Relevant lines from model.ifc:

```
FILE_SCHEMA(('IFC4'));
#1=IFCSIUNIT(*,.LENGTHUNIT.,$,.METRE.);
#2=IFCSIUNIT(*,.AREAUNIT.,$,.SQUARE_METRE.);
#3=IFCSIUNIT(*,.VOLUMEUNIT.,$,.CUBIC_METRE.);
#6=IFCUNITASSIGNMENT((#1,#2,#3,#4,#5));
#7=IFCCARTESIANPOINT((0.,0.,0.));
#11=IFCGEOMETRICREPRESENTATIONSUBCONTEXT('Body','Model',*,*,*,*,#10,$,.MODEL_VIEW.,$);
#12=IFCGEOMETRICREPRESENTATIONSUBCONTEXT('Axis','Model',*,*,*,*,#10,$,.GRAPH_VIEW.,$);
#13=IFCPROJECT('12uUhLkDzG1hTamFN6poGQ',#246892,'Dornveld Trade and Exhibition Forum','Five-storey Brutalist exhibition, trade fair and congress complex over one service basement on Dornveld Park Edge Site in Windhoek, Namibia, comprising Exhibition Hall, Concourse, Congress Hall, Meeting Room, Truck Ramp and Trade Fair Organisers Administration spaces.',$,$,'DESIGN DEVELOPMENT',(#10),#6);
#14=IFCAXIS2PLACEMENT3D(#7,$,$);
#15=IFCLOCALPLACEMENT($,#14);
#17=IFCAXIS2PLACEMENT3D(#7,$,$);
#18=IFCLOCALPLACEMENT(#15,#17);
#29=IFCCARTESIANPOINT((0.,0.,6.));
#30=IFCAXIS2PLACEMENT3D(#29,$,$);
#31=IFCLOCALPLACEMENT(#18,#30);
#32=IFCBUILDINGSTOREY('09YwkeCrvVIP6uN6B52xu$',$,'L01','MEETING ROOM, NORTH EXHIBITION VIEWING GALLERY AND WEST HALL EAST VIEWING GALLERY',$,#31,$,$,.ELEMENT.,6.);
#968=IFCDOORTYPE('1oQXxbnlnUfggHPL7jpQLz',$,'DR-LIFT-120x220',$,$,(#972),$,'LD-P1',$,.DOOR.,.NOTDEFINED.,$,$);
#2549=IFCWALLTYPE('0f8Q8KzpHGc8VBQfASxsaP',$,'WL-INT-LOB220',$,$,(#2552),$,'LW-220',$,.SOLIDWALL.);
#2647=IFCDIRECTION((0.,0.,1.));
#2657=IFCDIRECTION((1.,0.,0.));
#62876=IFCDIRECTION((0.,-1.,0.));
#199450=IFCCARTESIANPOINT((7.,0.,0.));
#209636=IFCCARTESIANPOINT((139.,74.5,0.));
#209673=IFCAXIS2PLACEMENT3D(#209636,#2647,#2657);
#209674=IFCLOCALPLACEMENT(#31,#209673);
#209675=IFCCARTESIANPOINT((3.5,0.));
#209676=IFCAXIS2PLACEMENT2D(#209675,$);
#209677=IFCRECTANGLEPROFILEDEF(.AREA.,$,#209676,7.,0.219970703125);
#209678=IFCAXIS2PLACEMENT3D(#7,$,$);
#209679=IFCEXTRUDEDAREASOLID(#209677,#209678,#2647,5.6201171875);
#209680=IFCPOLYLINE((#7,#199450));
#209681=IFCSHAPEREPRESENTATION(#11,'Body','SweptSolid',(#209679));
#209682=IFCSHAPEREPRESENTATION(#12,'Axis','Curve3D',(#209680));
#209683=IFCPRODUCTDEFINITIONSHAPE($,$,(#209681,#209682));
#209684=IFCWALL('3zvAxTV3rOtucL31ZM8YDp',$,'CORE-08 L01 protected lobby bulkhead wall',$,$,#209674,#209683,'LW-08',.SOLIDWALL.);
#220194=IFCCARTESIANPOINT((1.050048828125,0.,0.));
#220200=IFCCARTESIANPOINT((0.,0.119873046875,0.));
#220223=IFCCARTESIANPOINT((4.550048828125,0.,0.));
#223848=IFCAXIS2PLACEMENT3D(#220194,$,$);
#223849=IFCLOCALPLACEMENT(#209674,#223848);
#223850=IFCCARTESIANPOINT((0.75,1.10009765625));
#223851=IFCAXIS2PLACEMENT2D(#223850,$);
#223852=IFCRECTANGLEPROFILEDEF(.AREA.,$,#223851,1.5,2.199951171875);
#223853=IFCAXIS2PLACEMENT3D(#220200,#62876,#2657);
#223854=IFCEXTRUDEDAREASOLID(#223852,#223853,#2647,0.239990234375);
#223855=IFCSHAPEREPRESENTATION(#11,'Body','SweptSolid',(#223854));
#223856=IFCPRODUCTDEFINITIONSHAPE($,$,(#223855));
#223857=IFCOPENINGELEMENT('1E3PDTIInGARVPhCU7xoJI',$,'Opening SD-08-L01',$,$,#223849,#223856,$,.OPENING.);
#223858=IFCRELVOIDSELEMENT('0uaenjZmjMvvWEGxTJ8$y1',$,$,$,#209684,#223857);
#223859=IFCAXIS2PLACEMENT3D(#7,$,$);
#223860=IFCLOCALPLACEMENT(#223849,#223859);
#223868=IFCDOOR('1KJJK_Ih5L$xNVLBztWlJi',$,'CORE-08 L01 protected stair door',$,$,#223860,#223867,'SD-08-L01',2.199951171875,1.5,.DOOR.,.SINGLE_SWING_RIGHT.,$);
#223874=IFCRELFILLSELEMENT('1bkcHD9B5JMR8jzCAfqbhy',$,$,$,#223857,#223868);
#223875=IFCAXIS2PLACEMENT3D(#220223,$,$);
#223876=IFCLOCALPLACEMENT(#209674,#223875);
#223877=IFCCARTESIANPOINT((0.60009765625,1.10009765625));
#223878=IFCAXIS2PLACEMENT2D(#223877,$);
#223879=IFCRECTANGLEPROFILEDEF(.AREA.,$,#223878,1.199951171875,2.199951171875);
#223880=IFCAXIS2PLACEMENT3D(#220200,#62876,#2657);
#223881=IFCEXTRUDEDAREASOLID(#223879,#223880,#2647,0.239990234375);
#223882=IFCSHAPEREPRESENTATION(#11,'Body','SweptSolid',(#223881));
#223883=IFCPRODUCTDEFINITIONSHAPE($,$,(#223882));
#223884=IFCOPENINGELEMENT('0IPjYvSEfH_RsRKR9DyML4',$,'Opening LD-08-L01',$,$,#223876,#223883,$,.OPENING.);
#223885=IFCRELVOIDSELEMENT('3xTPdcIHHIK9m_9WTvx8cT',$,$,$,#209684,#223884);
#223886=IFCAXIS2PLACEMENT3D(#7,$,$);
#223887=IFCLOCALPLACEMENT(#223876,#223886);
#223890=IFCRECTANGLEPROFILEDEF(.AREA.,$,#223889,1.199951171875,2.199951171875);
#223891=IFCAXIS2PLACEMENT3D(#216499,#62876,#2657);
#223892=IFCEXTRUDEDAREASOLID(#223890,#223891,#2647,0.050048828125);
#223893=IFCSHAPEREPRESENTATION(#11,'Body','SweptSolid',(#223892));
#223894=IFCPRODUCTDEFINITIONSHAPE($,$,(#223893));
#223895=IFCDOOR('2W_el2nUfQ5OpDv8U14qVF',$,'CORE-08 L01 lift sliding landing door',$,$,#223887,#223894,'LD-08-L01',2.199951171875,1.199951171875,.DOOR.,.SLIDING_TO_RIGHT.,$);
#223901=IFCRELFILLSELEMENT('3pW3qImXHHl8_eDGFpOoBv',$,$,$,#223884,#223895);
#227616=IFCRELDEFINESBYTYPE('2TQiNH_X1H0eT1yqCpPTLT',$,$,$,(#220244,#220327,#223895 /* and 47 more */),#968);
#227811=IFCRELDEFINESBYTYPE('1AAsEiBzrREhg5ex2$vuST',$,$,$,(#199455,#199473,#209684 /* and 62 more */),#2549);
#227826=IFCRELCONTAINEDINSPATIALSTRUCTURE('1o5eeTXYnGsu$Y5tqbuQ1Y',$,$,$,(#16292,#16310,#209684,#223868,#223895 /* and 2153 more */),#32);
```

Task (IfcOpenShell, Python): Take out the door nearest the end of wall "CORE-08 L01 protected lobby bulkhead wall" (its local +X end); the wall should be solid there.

```python
import ifcopenshell
import ifcopenshell.api.feature
import ifcopenshell.api.root
import ifcopenshell.geom
import ifcopenshell.util.shape

model = ifcopenshell.open("model.ifc")
settings = ifcopenshell.geom.settings()


def volume(element):
    """Net volume in cubic metres, openings subtracted."""
    shape = ifcopenshell.geom.create_shape(settings, element)
    return ifcopenshell.util.shape.get_volume(shape.geometry)


door = model.by_guid("2W_el2nUfQ5OpDv8U14qVF")
opening = door.FillsVoids[0].RelatingOpeningElement
wall = opening.VoidsElements[0].RelatingBuildingElement
before = volume(wall)

ifcopenshell.api.root.remove_product(model, product=door)
ifcopenshell.api.feature.remove_feature(model, feature=opening)

after = volume(wall)

print(f"wall volume {before:.3f} -> {after:.3f} m3")

model.write("model_v2.ifc")
```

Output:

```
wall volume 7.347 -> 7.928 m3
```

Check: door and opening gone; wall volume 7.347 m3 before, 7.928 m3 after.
